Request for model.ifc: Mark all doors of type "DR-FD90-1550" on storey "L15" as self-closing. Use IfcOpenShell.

First a look at what the model holds.

```python
import ifcopenshell
import ifcopenshell.util.element

model = ifcopenshell.open("model.ifc")
print(model.schema)
storey = next(s for s in model.by_type("IfcBuildingStorey") if s.Name == "L15")
doors = [e for e in ifcopenshell.util.element.get_decomposition(storey) if e.is_a("IfcDoor")]
seen = {}
for e in doors:
    element_type = ifcopenshell.util.element.get_type(e)
    key = (element_type.Name if element_type != e and element_type else None, ifcopenshell.util.element.get_pset(e, "Pset_DoorCommon", "SelfClosing"))
    seen[key] = seen.get(key, 0) + 1
for (name, value), count in sorted(seen.items(), key=str):
    print(count, "x", name, "|", value)
```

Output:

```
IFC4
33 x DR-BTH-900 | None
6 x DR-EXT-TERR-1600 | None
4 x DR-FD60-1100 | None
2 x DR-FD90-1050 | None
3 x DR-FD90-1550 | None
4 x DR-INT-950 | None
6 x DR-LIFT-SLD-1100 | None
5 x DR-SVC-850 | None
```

```python
import ifcopenshell
import ifcopenshell.api.pset
import ifcopenshell.util.element

model = ifcopenshell.open("model.ifc")

storey = next(s for s in model.by_type("IfcBuildingStorey") if s.Name == "L15")
doors = [e for e in ifcopenshell.util.element.get_decomposition(storey) if e.is_a("IfcDoor")]

count = 0
for e in doors:
    element_type = ifcopenshell.util.element.get_type(e)
    if element_type in (None, e) or element_type.Name != "DR-FD90-1550":
        continue
    found = ifcopenshell.util.element.get_pset(e, "Pset_DoorCommon", should_inherit=False)
    if found:
        pset = model.by_id(found["id"])
        if len(ifcopenshell.util.element.get_elements_by_pset(pset)) > 1:
            pset = ifcopenshell.api.pset.unshare_pset(model, products=[e], pset=pset)[0]
    else:
        pset = ifcopenshell.api.pset.add_pset(model, product=e, name="Pset_DoorCommon")
    ifcopenshell.api.pset.edit_pset(model, pset=pset, properties={"SelfClosing": True})
    count += 1

print(count, "doors updated")

model.write("model_v2.ifc")
```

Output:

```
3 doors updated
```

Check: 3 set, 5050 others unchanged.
